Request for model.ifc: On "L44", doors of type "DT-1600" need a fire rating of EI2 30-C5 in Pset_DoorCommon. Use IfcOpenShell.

First a look at what the model holds.

```python
import ifcopenshell
import ifcopenshell.util.element

model = ifcopenshell.open("model.ifc")
print(model.schema)
storey = next(s for s in model.by_type("IfcBuildingStorey") if s.Name == "L44")
doors = [e for e in ifcopenshell.util.element.get_decomposition(storey) if e.is_a("IfcDoor")]
seen = {}
for e in doors:
    element_type = ifcopenshell.util.element.get_type(e)
    key = (element_type.Name if element_type != e and element_type else None, ifcopenshell.util.element.get_pset(e, "Pset_DoorCommon", "FireRating"))
    seen[key] = seen.get(key, 0) + 1
for (name, value), count in sorted(seen.items(), key=str):
    print(count, "x", name, "|", value)
```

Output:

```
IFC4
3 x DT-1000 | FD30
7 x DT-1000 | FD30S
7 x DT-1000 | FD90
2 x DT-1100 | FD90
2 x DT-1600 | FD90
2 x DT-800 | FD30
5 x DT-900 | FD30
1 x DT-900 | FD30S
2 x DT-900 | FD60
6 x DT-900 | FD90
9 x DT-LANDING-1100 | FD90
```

```python
import ifcopenshell
import ifcopenshell.api.pset
import ifcopenshell.util.element

model = ifcopenshell.open("model.ifc")

storey = next(s for s in model.by_type("IfcBuildingStorey") if s.Name == "L44")
doors = [e for e in ifcopenshell.util.element.get_decomposition(storey) if e.is_a("IfcDoor")]

count = 0
for e in doors:
    element_type = ifcopenshell.util.element.get_type(e)
    if element_type in (None, e) or element_type.Name != "DT-1600":
        continue
    # add_pset returns the element's existing set when there is one.
    pset = ifcopenshell.api.pset.add_pset(model, product=e, name="Pset_DoorCommon")
    ifcopenshell.api.pset.edit_pset(model, pset=pset, properties={"FireRating": "EI2 30-C5"})
    count += 1

print(count, "doors updated")

model.write("model_v2.ifc")
```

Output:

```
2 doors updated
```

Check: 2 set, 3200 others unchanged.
